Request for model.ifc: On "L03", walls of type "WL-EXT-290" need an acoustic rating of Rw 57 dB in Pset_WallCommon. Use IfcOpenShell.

First a look at what the model holds.

```python
import ifcopenshell
import ifcopenshell.util.element

model = ifcopenshell.open("model.ifc")
print(model.schema)
storey = next(s for s in model.by_type("IfcBuildingStorey") if s.Name == "L03")
walls = [e for e in ifcopenshell.util.element.get_decomposition(storey) if e.is_a("IfcWall")]
seen = {}
for e in walls:
    element_type = ifcopenshell.util.element.get_type(e)
    key = (element_type.Name if element_type != e and element_type else None, ifcopenshell.util.element.get_pset(e, "Pset_WallCommon", "AcousticRating"))
    seen[key] = seen.get(key, 0) + 1
for (name, value), count in sorted(seen.items(), key=str):
    print(count, "x", name, "|", value)
```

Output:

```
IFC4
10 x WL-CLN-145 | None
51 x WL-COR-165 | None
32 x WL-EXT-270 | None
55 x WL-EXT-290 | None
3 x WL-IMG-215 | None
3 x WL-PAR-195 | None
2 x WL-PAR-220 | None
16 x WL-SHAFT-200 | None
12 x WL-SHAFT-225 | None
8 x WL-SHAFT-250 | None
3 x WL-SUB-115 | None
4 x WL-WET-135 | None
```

```python
import ifcopenshell
import ifcopenshell.api.pset
import ifcopenshell.util.element

model = ifcopenshell.open("model.ifc")

storey = next(s for s in model.by_type("IfcBuildingStorey") if s.Name == "L03")
walls = [e for e in ifcopenshell.util.element.get_decomposition(storey) if e.is_a("IfcWall")]

count = 0
for e in walls:
    element_type = ifcopenshell.util.element.get_type(e)
    if element_type in (None, e) or element_type.Name != "WL-EXT-290":
        continue
    # add_pset returns the element's existing set when there is one.
    pset = ifcopenshell.api.pset.add_pset(model, product=e, name="Pset_WallCommon")
    ifcopenshell.api.pset.edit_pset(model, pset=pset, properties={"AcousticRating": "Rw 57 dB"})
    count += 1

print(count, "walls updated")

model.write("model_edited.ifc")
```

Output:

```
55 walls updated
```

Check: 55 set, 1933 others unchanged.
